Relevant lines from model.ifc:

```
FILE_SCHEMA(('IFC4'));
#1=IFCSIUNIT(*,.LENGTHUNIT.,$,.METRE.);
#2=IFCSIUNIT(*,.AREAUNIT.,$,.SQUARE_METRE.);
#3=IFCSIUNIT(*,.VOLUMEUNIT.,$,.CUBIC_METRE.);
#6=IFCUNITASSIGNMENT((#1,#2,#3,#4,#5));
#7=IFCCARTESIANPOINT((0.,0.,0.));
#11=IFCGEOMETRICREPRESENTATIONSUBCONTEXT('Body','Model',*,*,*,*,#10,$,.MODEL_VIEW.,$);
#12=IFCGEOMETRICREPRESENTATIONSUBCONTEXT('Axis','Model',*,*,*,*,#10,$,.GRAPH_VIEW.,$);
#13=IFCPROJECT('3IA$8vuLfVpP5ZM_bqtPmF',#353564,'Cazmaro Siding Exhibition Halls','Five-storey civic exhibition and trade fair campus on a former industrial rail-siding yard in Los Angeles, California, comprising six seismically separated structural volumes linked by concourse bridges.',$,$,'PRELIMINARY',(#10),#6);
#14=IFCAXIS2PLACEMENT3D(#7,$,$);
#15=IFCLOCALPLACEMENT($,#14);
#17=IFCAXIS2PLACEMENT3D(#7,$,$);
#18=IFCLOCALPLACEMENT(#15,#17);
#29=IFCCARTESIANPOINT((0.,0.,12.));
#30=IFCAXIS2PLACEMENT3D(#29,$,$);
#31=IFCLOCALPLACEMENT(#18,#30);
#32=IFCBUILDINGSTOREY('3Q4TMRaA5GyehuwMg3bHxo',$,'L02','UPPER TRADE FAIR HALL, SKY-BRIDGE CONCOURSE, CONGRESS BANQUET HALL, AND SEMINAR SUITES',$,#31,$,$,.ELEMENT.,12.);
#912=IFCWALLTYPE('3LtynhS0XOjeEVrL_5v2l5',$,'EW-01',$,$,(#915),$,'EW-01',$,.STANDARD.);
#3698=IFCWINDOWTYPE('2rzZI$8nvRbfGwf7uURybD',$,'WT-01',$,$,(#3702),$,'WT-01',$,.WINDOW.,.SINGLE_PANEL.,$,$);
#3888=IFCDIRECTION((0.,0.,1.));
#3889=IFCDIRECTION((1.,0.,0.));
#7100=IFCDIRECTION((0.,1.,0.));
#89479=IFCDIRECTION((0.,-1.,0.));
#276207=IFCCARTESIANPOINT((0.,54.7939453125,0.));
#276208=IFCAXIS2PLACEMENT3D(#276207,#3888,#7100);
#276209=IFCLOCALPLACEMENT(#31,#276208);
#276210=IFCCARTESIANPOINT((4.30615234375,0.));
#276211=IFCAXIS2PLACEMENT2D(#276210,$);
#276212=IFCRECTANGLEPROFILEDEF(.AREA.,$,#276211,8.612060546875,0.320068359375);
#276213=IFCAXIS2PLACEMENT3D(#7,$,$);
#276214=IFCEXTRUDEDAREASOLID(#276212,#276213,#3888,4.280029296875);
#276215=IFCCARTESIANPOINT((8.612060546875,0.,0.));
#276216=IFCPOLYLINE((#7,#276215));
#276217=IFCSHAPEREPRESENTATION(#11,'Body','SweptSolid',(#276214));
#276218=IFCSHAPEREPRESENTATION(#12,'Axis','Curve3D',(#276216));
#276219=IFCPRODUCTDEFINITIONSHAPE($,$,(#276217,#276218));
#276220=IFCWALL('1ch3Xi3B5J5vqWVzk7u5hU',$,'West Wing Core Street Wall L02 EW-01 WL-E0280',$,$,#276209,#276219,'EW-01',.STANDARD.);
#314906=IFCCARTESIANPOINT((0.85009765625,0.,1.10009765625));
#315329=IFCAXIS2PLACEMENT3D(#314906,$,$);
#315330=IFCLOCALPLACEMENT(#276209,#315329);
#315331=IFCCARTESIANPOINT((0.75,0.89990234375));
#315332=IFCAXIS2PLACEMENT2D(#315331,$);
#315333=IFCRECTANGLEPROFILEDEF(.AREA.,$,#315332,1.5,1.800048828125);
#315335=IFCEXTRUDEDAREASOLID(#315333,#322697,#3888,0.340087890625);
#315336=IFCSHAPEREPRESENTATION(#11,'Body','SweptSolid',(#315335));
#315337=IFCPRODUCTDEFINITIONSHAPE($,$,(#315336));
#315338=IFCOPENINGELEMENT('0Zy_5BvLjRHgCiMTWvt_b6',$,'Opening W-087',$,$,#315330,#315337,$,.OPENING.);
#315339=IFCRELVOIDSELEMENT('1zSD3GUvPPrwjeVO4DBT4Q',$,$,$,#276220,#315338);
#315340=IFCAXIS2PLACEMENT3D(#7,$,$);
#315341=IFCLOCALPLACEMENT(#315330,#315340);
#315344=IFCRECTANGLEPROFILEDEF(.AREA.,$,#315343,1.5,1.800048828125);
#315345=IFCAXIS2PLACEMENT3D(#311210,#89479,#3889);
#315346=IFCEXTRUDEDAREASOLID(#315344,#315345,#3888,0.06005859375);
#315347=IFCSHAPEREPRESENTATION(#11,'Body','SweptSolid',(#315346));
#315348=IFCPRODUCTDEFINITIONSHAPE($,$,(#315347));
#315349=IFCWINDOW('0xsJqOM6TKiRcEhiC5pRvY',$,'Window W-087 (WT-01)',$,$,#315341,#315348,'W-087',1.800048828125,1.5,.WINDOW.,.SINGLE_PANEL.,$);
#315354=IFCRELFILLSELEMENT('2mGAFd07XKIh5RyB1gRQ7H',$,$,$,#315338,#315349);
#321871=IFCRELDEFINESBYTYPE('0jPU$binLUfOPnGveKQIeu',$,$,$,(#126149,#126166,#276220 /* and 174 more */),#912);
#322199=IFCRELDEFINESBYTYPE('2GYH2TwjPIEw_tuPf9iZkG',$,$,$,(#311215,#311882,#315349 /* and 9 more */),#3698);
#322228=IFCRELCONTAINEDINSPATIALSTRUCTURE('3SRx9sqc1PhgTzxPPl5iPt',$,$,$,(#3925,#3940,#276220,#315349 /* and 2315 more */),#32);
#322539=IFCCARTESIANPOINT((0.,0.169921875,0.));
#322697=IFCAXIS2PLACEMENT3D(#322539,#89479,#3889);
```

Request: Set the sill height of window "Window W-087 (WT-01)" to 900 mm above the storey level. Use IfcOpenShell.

```python
import numpy as np
import ifcopenshell
import ifcopenshell.api.geometry
import ifcopenshell.geom
import ifcopenshell.util.element
import ifcopenshell.util.placement
import ifcopenshell.util.shape
import ifcopenshell.util.unit

model = ifcopenshell.open("model.ifc")
unit_scale = ifcopenshell.util.unit.calculate_unit_scale(model)

window = model.by_guid("0xsJqOM6TKiRcEhiC5pRvY")
opening = window.FillsVoids[0].RelatingOpeningElement
storey = ifcopenshell.util.element.get_container(window, ifc_class="IfcBuildingStorey")
level = ifcopenshell.util.placement.get_local_placement(storey.ObjectPlacement)[2, 3]

# The opening's origin need not be at the sill, so measure its lowest point.
shape = ifcopenshell.geom.create_shape(ifcopenshell.geom.settings(), opening)
bottom = ifcopenshell.util.shape.get_shape_bottom_elevation(shape, shape.geometry) / unit_scale
dz = level + 0.9 / unit_scale - bottom

shift = np.array([0.0, 0.0, dz])
# The window is placed relative to its opening, so it follows when the opening moves.
matrix = ifcopenshell.util.placement.get_local_placement(opening.ObjectPlacement)
matrix[:3, 3] += shift
ifcopenshell.api.geometry.edit_object_placement(
    model, product=opening, matrix=matrix, is_si=False, should_transform_children=True
)

print(f"moved by {dz * unit_scale:+.3f} m")

model.write("model_edited.ifc")
```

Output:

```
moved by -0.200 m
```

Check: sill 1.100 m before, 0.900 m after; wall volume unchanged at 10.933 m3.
